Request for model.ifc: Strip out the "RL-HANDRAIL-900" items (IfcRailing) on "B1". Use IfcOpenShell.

First a look at what the model holds.

```python
import ifcopenshell
import ifcopenshell.util.element

model = ifcopenshell.open("model.ifc")
print(model.schema)
storey = next(s for s in model.by_type("IfcBuildingStorey") if s.Name == "B1")
railings = [e for e in ifcopenshell.util.element.get_decomposition(storey) if e.is_a("IfcRailing")]
seen = {}
for e in railings:
    element_type = ifcopenshell.util.element.get_type(e)
    name = element_type.Name if element_type not in (None, e) else None
    seen[name] = seen.get(name, 0) + 1
for name, count in sorted(seen.items(), key=str):
    print(count, "x", name)
```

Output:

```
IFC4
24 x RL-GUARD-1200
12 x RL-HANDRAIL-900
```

```python
import ifcopenshell
import ifcopenshell.api.root
import ifcopenshell.util.element

model = ifcopenshell.open("model.ifc")

storey = next(s for s in model.by_type("IfcBuildingStorey") if s.Name == "B1")
railings = [e for e in ifcopenshell.util.element.get_decomposition(storey) if e.is_a("IfcRailing")]
targets = [e for e in railings if (t := ifcopenshell.util.element.get_type(e)) not in (None, e) and t.Name == "RL-HANDRAIL-900"]

for e in targets:
    ifcopenshell.api.root.remove_product(model, product=e)
print(len(targets), "removed")

model.write("model_updated.ifc")
```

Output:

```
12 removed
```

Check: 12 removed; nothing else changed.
